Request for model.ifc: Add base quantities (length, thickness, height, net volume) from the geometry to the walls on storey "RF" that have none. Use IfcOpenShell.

First a look at what the model holds.

```python
import ifcopenshell
import ifcopenshell.util.element
import ifcopenshell.util.unit

model = ifcopenshell.open("model.ifc")
print(model.schema)
for unit_type in ("LENGTHUNIT", "AREAUNIT", "VOLUMEUNIT"):
    print(unit_type, ifcopenshell.util.unit.calculate_unit_scale(model, unit_type))
storey = next(s for s in model.by_type("IfcBuildingStorey") if s.Name == "RF")
walls = [e for e in ifcopenshell.util.element.get_decomposition(storey) if e.is_a("IfcWall")]
for e in sorted(walls, key=lambda e: e.id()):
    print(e.id(), e.is_a(), e.Name, list(ifcopenshell.util.element.get_psets(e, qtos_only=True)), sep=" | ")
```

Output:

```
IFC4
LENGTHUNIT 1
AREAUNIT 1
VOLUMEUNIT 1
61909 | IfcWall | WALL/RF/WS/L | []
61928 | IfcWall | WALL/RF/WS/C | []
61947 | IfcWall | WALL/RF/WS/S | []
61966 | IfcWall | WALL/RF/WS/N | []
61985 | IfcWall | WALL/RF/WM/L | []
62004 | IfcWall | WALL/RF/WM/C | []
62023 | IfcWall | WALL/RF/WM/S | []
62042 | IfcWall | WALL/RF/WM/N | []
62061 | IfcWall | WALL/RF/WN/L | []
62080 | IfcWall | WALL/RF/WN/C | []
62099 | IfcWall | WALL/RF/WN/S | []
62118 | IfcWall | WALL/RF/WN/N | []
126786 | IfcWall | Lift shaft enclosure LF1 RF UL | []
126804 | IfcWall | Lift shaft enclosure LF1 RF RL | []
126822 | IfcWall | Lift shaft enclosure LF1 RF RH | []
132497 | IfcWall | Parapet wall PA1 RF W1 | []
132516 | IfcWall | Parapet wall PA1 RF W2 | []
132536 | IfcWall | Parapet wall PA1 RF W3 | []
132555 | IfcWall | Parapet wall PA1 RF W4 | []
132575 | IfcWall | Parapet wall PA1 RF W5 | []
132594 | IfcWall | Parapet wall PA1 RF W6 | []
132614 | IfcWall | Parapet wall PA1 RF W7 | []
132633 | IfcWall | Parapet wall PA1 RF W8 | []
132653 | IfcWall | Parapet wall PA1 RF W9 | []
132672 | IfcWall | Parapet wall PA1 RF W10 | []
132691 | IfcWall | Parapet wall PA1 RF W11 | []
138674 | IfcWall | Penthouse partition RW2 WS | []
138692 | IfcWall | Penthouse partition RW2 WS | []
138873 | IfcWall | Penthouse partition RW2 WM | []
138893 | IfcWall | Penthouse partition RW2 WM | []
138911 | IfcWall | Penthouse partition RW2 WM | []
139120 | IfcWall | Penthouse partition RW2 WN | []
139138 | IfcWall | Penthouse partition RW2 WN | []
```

```python
import ifcopenshell
import ifcopenshell.api.pset
import ifcopenshell.geom
import ifcopenshell.util.element
import ifcopenshell.util.shape
import ifcopenshell.util.unit

model = ifcopenshell.open("model.ifc")
unit_scale = ifcopenshell.util.unit.calculate_unit_scale(model)
volume_scale = ifcopenshell.util.unit.calculate_unit_scale(model, "VOLUMEUNIT")
settings = ifcopenshell.geom.settings()

storey = next(s for s in model.by_type("IfcBuildingStorey") if s.Name == "RF")
walls = [e for e in ifcopenshell.util.element.get_decomposition(storey) if e.is_a("IfcWall")]

for e in sorted(walls, key=lambda e: e.id()):
    if ifcopenshell.util.element.get_psets(e, qtos_only=True, should_inherit=False):
        continue
    # Geometry comes back in metres, in the element's own axes.
    shape = ifcopenshell.geom.create_shape(settings, e)
    values = {
        "Length": ifcopenshell.util.shape.get_x(shape.geometry) / unit_scale,
        "Width": ifcopenshell.util.shape.get_y(shape.geometry) / unit_scale,
        "Height": ifcopenshell.util.shape.get_z(shape.geometry) / unit_scale,
        "NetVolume": ifcopenshell.util.shape.get_volume(shape.geometry) / volume_scale,
    }
    qto = ifcopenshell.api.pset.add_qto(model, product=e, name="Qto_WallBaseQuantities")
    ifcopenshell.api.pset.edit_qto(model, qto=qto, properties=values)
    print(e.id(), {k: round(v, 3) for k, v in values.items()})

model.write("model-out.ifc")
```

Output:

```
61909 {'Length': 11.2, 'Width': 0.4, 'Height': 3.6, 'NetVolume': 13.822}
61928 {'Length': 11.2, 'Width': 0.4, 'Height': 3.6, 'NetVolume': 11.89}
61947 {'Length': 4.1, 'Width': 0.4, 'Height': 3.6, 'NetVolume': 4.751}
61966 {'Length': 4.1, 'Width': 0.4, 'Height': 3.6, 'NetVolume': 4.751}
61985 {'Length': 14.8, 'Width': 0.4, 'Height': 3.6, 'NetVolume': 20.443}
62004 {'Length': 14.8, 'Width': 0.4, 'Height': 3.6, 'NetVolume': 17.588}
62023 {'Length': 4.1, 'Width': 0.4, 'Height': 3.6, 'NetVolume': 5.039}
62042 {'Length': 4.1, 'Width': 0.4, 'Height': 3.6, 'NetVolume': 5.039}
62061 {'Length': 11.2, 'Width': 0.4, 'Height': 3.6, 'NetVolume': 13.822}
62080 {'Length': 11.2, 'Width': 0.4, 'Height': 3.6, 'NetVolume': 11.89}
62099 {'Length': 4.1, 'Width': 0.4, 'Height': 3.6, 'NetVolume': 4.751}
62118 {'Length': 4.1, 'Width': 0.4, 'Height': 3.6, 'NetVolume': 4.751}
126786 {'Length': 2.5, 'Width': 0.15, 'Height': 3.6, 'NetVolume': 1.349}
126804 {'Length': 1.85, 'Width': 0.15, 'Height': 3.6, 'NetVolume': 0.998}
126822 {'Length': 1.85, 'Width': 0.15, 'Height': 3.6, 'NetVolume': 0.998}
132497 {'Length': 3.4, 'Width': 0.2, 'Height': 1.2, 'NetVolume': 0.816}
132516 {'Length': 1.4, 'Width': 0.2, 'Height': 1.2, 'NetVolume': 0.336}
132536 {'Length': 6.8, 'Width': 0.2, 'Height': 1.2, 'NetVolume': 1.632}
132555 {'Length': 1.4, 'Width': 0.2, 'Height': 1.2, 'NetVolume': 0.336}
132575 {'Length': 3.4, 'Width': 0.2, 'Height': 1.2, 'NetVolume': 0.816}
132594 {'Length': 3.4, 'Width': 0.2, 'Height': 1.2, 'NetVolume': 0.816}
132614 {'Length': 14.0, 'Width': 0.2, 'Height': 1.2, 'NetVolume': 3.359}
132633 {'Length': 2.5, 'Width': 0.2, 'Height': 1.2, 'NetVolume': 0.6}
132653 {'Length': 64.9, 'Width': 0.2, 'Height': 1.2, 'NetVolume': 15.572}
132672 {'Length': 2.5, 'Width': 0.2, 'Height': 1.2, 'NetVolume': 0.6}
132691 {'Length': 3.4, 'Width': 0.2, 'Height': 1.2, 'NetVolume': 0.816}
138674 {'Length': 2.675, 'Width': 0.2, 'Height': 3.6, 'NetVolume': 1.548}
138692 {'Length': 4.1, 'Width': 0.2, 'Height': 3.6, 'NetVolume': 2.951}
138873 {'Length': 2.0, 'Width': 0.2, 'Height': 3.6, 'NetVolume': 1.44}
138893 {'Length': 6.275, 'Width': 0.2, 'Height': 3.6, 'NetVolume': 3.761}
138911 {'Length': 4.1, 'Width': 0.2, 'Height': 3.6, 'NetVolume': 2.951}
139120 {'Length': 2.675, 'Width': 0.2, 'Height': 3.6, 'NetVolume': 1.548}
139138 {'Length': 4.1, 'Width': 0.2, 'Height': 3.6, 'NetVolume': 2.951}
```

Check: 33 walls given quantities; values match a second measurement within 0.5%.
